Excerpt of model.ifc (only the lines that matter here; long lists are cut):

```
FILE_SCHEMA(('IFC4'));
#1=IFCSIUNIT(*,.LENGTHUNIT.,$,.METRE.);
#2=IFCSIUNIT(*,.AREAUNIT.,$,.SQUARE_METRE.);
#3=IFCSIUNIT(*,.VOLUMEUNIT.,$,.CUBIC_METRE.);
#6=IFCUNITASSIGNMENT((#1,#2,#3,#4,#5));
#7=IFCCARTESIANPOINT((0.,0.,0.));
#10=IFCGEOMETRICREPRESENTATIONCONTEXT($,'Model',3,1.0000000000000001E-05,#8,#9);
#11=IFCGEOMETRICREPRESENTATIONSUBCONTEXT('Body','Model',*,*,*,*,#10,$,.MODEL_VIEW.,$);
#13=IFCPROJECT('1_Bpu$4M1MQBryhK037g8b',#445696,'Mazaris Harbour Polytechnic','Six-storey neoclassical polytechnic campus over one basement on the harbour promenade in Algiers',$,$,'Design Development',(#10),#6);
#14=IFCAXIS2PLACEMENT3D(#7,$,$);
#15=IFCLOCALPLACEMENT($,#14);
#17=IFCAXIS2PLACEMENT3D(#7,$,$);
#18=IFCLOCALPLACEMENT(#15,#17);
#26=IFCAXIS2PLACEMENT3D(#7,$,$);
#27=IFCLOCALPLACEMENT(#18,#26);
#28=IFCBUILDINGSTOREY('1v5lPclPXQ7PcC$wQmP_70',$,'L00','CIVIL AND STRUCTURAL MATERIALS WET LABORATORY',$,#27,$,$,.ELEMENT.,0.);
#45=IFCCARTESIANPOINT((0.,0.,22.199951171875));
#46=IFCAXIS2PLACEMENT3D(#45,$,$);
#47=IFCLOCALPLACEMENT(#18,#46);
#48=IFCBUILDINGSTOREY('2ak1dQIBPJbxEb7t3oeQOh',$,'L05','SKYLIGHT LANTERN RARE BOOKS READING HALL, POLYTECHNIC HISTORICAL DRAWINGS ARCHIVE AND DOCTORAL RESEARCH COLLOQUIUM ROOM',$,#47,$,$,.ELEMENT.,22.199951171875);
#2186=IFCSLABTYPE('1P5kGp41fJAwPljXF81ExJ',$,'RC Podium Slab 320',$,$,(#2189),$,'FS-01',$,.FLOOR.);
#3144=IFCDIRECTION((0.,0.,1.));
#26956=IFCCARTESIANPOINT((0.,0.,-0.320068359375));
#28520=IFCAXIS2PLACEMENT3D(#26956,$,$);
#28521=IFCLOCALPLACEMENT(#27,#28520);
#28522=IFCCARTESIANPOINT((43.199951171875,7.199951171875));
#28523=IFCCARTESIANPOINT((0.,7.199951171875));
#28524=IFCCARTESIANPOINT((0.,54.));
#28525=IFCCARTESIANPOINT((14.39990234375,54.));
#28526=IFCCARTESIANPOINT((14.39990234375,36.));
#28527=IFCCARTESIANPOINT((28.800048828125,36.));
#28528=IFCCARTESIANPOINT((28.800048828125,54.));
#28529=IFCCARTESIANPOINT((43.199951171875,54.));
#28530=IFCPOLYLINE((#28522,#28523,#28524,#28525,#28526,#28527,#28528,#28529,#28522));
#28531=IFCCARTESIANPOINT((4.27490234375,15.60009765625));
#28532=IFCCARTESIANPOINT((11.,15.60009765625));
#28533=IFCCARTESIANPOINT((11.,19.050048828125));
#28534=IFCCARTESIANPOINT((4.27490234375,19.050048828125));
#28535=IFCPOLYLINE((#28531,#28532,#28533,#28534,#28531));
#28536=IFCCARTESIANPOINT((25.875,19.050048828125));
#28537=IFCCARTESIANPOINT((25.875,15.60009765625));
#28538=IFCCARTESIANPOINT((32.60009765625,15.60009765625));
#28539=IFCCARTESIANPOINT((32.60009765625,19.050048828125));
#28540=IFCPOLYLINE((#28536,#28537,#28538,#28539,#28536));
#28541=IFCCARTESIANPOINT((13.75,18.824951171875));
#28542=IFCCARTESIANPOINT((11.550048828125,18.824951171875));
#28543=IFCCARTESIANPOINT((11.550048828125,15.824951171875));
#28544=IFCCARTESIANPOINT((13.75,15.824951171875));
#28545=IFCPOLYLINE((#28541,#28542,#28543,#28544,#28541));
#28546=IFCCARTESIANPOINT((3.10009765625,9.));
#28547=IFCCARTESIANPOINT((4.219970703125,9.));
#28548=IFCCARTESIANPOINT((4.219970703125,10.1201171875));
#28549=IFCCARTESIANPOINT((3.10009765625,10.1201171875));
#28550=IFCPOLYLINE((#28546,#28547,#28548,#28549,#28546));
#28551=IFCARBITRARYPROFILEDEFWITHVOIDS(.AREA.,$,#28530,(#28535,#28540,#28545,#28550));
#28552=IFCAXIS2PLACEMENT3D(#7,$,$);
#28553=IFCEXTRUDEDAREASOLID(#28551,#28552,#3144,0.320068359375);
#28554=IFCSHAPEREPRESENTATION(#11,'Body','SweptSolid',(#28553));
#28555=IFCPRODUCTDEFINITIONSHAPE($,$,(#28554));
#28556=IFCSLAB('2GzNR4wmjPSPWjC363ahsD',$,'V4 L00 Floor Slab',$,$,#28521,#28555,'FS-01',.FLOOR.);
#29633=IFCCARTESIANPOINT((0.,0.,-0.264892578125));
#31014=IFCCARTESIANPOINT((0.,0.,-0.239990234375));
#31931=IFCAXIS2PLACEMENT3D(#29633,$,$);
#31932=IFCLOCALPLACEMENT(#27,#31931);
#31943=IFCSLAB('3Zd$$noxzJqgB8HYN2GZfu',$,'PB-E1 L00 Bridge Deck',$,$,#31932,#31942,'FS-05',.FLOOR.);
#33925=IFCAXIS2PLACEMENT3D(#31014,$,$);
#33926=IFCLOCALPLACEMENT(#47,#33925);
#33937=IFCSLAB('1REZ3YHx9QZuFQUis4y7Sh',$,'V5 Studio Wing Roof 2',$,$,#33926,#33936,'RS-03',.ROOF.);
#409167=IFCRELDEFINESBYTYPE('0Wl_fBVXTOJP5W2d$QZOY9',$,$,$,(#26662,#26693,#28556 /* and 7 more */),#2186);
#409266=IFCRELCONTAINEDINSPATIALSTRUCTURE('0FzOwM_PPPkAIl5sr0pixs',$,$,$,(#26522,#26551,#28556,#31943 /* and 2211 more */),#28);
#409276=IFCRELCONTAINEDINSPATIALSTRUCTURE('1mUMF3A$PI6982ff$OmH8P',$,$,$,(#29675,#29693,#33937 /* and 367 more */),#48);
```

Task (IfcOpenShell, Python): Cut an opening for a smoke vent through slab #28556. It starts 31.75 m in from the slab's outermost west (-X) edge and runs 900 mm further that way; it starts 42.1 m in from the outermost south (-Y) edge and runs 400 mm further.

```python
import numpy as np
import ifcopenshell
import ifcopenshell.api.feature
import ifcopenshell.api.geometry
import ifcopenshell.api.root
import ifcopenshell.geom
import ifcopenshell.util.placement
import ifcopenshell.util.representation
import ifcopenshell.util.shape
import ifcopenshell.util.unit

model = ifcopenshell.open("model.ifc")
unit_scale = ifcopenshell.util.unit.calculate_unit_scale(model)
settings = ifcopenshell.geom.settings()


def volume(element):
    """Net volume in cubic metres, openings subtracted."""
    shape = ifcopenshell.geom.create_shape(settings, element)
    return ifcopenshell.util.shape.get_volume(shape.geometry)


slab = model.by_id(28556)
before = volume(slab)

# Extent in the slab's own axes, in metres. The edges named are its -X and -Y sides.
slab_shape = ifcopenshell.geom.create_shape(settings, slab)
vertices = ifcopenshell.util.shape.get_vertices(slab_shape.geometry)
x_min, y_min, bottom = vertices.min(axis=0)
top = vertices[:, 2].max()

opening = ifcopenshell.api.root.create_entity(model, ifc_class="IfcOpeningElement", name="Smoke vent opening", predefined_type="OPENING")
context = ifcopenshell.util.representation.get_context(model, "Model", "Body", "MODEL_VIEW")
width, depth = 0.9, 0.4
outline = [(0.0, 0.0), (width, 0.0), (width, depth), (0.0, depth), (0.0, 0.0)]
# Overshoot both faces by 50 mm so the cut is clean.
shape = ifcopenshell.api.geometry.add_slab_representation(
    model, context=context, depth=top - bottom + 0.1, polyline=outline
)
ifcopenshell.api.geometry.assign_representation(model, product=opening, representation=shape)

matrix = ifcopenshell.util.placement.get_local_placement(slab.ObjectPlacement)
matrix[:, 3] = matrix @ np.append(np.array([x_min + 31.75, y_min + 42.1, bottom - 0.05]) / unit_scale, 1.0)
ifcopenshell.api.geometry.edit_object_placement(model, product=opening, matrix=matrix, is_si=False)
ifcopenshell.api.feature.add_feature(model, feature=opening, element=slab)

after = volume(slab)

print(f"slab volume {before:.3f} -> {after:.3f} m3")

model.write("model_edited.ifc")
```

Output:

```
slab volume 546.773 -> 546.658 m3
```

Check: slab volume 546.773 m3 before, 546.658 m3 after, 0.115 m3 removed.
